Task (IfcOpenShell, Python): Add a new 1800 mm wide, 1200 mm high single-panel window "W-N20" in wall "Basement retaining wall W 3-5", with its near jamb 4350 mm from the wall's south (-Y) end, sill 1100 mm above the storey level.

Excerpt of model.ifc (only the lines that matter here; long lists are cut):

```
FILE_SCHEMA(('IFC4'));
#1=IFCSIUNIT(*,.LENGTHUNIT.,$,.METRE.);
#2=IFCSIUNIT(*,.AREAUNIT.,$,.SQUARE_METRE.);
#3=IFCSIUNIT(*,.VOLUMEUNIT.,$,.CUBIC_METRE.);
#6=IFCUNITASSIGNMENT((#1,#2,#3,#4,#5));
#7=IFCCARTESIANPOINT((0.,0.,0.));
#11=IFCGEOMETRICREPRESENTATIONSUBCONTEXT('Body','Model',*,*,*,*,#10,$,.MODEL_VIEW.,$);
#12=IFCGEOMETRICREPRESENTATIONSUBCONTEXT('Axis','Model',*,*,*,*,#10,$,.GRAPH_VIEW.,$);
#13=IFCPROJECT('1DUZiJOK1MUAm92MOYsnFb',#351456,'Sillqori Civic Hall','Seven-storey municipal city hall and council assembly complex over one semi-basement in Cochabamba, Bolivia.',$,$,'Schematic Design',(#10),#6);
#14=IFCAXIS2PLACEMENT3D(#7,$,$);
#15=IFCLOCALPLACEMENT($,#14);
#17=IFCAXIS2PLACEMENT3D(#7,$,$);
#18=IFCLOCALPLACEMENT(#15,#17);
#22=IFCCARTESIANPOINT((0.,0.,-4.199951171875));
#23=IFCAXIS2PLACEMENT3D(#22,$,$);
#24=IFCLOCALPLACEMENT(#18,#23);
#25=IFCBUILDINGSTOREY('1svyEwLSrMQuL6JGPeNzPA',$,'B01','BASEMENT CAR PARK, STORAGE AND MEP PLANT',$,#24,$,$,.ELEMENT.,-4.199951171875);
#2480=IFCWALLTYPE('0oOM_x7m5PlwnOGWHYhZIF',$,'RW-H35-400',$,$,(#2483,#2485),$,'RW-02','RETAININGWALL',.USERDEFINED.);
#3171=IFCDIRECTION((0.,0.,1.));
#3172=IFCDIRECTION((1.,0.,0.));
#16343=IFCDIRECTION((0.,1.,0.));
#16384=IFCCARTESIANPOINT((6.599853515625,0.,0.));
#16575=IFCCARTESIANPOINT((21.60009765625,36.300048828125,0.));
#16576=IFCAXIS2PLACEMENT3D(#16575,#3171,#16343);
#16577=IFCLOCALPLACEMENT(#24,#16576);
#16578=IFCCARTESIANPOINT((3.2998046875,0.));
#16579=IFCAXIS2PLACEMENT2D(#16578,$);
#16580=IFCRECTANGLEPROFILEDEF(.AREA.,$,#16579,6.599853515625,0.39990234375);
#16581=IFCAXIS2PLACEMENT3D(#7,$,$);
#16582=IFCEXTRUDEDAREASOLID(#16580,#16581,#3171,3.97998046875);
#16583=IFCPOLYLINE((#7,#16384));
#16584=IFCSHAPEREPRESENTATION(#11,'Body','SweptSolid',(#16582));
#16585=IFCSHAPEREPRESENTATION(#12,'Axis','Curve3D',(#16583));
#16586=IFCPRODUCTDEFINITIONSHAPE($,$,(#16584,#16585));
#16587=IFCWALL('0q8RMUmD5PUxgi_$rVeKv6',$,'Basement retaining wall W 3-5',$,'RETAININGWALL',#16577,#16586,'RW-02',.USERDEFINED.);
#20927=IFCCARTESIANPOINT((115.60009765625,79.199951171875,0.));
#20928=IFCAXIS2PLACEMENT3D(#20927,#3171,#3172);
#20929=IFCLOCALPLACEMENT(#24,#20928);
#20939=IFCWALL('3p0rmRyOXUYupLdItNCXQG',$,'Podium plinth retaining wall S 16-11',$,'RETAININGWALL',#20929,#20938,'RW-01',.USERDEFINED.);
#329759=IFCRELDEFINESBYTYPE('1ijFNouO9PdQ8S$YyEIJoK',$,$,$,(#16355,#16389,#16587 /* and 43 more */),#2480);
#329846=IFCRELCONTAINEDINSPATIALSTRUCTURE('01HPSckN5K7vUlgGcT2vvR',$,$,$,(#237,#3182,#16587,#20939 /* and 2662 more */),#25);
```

```python
import numpy as np
import ifcopenshell
import ifcopenshell.api.feature
import ifcopenshell.api.geometry
import ifcopenshell.api.root
import ifcopenshell.api.spatial
import ifcopenshell.geom
import ifcopenshell.util.element
import ifcopenshell.util.placement
import ifcopenshell.util.representation
import ifcopenshell.util.shape
import ifcopenshell.util.unit

model = ifcopenshell.open("model.ifc")
unit_scale = ifcopenshell.util.unit.calculate_unit_scale(model)
settings = ifcopenshell.geom.settings()


def volume(element):
    """Net volume in cubic metres, openings subtracted."""
    shape = ifcopenshell.geom.create_shape(settings, element)
    return ifcopenshell.util.shape.get_volume(shape.geometry)


wall = model.by_id(16587)
storey = ifcopenshell.util.element.get_container(wall, ifc_class="IfcBuildingStorey")
context = ifcopenshell.util.representation.get_context(model, "Model", "Body", "MODEL_VIEW")
before = volume(wall)

width, height, from_end, sill = 1.8, 1.2, 4.35, 1.1  # metres

# The wall runs along its own X axis, and the end named is its -X end.
wall_shape = ifcopenshell.geom.create_shape(settings, wall)
x, y, z = ifcopenshell.util.shape.get_vertices(wall_shape.geometry).T
start = x.min() + from_end
face, thickness = float(y.min()), float(y.max() - y.min())
wall_matrix = ifcopenshell.util.placement.get_local_placement(wall.ObjectPlacement)
level = ifcopenshell.util.placement.get_local_placement(storey.ObjectPlacement)[2, 3]


def in_wall(x, y):
    """Placement at x, y metres in the wall's axes, at sill height."""
    matrix = wall_matrix.copy()
    matrix[:, 3] = wall_matrix @ np.array([x / unit_scale, y / unit_scale, 0.0, 1.0])
    matrix[2, 3] = level + sill / unit_scale
    return matrix


# Opening: a box that overshoots both wall faces by 50 mm.
opening = ifcopenshell.api.root.create_entity(model, ifc_class="IfcOpeningElement", predefined_type="OPENING")
box = ifcopenshell.api.geometry.add_wall_representation(
    model, context=context, length=width, height=height, thickness=thickness + 0.1
)
ifcopenshell.api.geometry.assign_representation(model, product=opening, representation=box)
ifcopenshell.api.geometry.edit_object_placement(model, product=opening, matrix=in_wall(start, face - 0.05), is_si=False)
ifcopenshell.api.feature.add_feature(model, feature=opening, element=wall)

window = ifcopenshell.api.root.create_entity(model, ifc_class="IfcWindow", name="W-N20", predefined_type="WINDOW")
window.OverallWidth, window.OverallHeight = width / unit_scale, height / unit_scale
window.PartitioningType = "SINGLE_PANEL"
body = ifcopenshell.api.geometry.add_window_representation(
    model,
    context=context,
    overall_width=window.OverallWidth,
    overall_height=window.OverallHeight,
    partition_type="SINGLE_PANEL",
)
ifcopenshell.api.geometry.assign_representation(model, product=window, representation=body)
ifcopenshell.api.spatial.assign_container(model, products=[window], relating_structure=storey)
ifcopenshell.api.feature.add_filling(model, opening=opening, element=window)

# Centre the window in the wall's thickness.
ifcopenshell.api.geometry.edit_object_placement(model, product=window, matrix=in_wall(start, face), is_si=False)
window_shape = ifcopenshell.geom.create_shape(settings, window)
depth = ifcopenshell.util.shape.get_vertices(window_shape.geometry)[:, 1]
offset = face + thickness / 2 - (depth.min() + depth.max()) / 2
ifcopenshell.api.geometry.edit_object_placement(model, product=window, matrix=in_wall(start, offset), is_si=False)

after = volume(wall)

print(f"wall volume {before:.3f} -> {after:.3f} m3")

model.write("model_edited.ifc")
```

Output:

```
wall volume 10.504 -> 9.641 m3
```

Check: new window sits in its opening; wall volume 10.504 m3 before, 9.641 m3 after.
